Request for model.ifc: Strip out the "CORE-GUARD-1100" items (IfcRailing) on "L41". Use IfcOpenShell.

First a look at what the model holds.

```python
import ifcopenshell
import ifcopenshell.util.element

model = ifcopenshell.open("model.ifc")
print(model.schema)
storey = next(s for s in model.by_type("IfcBuildingStorey") if s.Name == "L41")
railings = [e for e in ifcopenshell.util.element.get_decomposition(storey) if e.is_a("IfcRailing")]
seen = {}
for e in railings:
    element_type = ifcopenshell.util.element.get_type(e)
    name = element_type.Name if element_type not in (None, e) else None
    seen[name] = seen.get(name, 0) + 1
for name, count in sorted(seen.items(), key=str):
    print(count, "x", name)
```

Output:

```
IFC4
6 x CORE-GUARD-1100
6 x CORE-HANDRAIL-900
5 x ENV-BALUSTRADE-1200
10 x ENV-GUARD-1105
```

```python
import ifcopenshell
import ifcopenshell.api.root
import ifcopenshell.util.element

model = ifcopenshell.open("model.ifc")

storey = next(s for s in model.by_type("IfcBuildingStorey") if s.Name == "L41")
railings = [e for e in ifcopenshell.util.element.get_decomposition(storey) if e.is_a("IfcRailing")]
targets = [e for e in railings if (t := ifcopenshell.util.element.get_type(e)) not in (None, e) and t.Name == "CORE-GUARD-1100"]

for e in targets:
    ifcopenshell.api.root.remove_product(model, product=e)
print(len(targets), "removed")

model.write("model-out.ifc")
```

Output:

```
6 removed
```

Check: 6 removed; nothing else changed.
